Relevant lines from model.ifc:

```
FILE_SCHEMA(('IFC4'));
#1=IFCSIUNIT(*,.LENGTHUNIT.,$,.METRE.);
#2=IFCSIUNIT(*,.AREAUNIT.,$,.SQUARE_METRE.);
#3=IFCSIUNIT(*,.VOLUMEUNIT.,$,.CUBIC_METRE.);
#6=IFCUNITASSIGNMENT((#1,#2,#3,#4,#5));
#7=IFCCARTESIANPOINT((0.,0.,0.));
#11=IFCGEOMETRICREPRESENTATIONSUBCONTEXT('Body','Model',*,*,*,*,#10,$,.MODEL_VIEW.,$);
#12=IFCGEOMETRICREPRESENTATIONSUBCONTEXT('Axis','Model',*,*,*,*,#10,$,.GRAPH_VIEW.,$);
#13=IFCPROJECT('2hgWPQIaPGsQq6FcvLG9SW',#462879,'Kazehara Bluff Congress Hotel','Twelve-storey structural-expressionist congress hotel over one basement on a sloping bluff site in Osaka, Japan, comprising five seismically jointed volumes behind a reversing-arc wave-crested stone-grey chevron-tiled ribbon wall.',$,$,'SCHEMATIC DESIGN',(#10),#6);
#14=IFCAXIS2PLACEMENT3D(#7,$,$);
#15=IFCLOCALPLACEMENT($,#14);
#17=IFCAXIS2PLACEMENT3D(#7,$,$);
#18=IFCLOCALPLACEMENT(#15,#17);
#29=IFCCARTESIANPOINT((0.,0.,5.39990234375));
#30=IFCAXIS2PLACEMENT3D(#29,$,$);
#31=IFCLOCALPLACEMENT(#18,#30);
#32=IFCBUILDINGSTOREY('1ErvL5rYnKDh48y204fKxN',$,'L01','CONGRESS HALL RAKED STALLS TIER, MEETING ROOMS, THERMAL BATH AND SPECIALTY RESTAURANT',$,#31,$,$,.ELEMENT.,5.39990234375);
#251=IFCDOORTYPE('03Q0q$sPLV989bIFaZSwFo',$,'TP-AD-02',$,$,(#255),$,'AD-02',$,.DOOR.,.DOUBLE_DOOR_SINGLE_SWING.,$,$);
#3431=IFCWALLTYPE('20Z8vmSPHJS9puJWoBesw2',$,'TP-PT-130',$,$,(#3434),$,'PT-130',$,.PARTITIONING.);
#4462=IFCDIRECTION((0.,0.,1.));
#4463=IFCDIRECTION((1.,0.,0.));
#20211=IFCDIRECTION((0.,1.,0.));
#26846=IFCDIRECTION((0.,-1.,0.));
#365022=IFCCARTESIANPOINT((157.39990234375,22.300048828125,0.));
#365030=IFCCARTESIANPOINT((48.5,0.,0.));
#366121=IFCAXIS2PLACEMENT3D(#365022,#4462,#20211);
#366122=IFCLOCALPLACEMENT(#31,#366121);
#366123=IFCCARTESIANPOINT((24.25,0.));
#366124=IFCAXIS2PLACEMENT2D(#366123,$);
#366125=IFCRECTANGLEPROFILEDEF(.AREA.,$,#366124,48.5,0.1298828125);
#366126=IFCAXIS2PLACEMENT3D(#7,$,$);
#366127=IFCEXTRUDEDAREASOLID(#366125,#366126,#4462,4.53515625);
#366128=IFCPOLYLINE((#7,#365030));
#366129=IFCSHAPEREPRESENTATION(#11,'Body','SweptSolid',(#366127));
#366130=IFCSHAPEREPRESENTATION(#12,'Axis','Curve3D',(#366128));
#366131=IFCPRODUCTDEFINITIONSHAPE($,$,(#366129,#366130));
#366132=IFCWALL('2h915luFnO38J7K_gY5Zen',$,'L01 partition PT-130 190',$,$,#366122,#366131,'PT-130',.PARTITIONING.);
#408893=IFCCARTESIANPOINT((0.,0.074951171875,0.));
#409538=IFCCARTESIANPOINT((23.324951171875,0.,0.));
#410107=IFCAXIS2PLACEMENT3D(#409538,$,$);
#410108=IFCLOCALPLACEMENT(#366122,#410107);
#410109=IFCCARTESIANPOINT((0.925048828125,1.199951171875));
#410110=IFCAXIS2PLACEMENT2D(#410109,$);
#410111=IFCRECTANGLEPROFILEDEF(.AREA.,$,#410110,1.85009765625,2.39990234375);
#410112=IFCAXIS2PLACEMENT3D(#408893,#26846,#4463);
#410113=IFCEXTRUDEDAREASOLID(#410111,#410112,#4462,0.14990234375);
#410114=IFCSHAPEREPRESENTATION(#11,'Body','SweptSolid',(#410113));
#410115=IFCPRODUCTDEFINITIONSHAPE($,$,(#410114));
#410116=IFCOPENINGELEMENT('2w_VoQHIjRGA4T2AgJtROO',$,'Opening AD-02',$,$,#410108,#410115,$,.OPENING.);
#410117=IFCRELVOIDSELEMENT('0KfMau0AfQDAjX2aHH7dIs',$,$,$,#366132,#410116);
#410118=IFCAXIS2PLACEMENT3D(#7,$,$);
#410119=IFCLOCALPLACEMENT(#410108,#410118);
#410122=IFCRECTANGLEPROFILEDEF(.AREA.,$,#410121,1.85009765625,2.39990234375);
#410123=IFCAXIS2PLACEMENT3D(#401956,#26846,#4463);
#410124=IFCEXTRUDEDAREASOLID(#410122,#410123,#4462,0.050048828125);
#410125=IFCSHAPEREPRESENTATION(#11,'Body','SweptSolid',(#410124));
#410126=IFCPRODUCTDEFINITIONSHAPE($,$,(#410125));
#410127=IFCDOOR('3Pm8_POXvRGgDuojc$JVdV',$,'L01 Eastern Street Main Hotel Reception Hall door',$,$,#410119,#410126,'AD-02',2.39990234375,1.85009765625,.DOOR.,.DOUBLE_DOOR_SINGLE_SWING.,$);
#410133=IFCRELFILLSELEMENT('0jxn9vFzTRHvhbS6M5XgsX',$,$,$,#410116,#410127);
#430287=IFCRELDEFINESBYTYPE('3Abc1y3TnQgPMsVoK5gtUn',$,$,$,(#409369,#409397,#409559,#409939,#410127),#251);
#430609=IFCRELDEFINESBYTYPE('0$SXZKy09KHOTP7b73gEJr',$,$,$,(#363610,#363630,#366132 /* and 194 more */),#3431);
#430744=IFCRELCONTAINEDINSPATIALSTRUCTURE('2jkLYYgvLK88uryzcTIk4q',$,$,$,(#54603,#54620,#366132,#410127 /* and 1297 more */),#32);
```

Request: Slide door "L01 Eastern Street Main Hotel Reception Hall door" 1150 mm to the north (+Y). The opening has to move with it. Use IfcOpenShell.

```python
import ifcopenshell
import ifcopenshell.api.geometry
import ifcopenshell.util.placement
import ifcopenshell.util.unit

model = ifcopenshell.open("model.ifc")
unit_scale = ifcopenshell.util.unit.calculate_unit_scale(model)

door = model.by_guid("3Pm8_POXvRGgDuojc$JVdV")
opening = door.FillsVoids[0].RelatingOpeningElement
wall = opening.VoidsElements[0].RelatingBuildingElement

wall_matrix = ifcopenshell.util.placement.get_local_placement(wall.ObjectPlacement)
shift = wall_matrix[:3, 0] * 1.15 / unit_scale
before = ifcopenshell.util.placement.get_local_placement(door.ObjectPlacement)[:3, 3].copy()

# The door is placed relative to its opening, so it follows when the opening moves.
matrix = ifcopenshell.util.placement.get_local_placement(opening.ObjectPlacement)
matrix[:3, 3] += shift
ifcopenshell.api.geometry.edit_object_placement(
    model, product=opening, matrix=matrix, is_si=False, should_transform_children=True
)

after = ifcopenshell.util.placement.get_local_placement(door.ObjectPlacement)[:3, 3]
print("door moved by", (after - before).round(3) + 0.0)

model.write("model_edited.ifc")
```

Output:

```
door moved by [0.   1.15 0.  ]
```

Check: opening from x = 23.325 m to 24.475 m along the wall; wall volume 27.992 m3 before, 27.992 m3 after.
